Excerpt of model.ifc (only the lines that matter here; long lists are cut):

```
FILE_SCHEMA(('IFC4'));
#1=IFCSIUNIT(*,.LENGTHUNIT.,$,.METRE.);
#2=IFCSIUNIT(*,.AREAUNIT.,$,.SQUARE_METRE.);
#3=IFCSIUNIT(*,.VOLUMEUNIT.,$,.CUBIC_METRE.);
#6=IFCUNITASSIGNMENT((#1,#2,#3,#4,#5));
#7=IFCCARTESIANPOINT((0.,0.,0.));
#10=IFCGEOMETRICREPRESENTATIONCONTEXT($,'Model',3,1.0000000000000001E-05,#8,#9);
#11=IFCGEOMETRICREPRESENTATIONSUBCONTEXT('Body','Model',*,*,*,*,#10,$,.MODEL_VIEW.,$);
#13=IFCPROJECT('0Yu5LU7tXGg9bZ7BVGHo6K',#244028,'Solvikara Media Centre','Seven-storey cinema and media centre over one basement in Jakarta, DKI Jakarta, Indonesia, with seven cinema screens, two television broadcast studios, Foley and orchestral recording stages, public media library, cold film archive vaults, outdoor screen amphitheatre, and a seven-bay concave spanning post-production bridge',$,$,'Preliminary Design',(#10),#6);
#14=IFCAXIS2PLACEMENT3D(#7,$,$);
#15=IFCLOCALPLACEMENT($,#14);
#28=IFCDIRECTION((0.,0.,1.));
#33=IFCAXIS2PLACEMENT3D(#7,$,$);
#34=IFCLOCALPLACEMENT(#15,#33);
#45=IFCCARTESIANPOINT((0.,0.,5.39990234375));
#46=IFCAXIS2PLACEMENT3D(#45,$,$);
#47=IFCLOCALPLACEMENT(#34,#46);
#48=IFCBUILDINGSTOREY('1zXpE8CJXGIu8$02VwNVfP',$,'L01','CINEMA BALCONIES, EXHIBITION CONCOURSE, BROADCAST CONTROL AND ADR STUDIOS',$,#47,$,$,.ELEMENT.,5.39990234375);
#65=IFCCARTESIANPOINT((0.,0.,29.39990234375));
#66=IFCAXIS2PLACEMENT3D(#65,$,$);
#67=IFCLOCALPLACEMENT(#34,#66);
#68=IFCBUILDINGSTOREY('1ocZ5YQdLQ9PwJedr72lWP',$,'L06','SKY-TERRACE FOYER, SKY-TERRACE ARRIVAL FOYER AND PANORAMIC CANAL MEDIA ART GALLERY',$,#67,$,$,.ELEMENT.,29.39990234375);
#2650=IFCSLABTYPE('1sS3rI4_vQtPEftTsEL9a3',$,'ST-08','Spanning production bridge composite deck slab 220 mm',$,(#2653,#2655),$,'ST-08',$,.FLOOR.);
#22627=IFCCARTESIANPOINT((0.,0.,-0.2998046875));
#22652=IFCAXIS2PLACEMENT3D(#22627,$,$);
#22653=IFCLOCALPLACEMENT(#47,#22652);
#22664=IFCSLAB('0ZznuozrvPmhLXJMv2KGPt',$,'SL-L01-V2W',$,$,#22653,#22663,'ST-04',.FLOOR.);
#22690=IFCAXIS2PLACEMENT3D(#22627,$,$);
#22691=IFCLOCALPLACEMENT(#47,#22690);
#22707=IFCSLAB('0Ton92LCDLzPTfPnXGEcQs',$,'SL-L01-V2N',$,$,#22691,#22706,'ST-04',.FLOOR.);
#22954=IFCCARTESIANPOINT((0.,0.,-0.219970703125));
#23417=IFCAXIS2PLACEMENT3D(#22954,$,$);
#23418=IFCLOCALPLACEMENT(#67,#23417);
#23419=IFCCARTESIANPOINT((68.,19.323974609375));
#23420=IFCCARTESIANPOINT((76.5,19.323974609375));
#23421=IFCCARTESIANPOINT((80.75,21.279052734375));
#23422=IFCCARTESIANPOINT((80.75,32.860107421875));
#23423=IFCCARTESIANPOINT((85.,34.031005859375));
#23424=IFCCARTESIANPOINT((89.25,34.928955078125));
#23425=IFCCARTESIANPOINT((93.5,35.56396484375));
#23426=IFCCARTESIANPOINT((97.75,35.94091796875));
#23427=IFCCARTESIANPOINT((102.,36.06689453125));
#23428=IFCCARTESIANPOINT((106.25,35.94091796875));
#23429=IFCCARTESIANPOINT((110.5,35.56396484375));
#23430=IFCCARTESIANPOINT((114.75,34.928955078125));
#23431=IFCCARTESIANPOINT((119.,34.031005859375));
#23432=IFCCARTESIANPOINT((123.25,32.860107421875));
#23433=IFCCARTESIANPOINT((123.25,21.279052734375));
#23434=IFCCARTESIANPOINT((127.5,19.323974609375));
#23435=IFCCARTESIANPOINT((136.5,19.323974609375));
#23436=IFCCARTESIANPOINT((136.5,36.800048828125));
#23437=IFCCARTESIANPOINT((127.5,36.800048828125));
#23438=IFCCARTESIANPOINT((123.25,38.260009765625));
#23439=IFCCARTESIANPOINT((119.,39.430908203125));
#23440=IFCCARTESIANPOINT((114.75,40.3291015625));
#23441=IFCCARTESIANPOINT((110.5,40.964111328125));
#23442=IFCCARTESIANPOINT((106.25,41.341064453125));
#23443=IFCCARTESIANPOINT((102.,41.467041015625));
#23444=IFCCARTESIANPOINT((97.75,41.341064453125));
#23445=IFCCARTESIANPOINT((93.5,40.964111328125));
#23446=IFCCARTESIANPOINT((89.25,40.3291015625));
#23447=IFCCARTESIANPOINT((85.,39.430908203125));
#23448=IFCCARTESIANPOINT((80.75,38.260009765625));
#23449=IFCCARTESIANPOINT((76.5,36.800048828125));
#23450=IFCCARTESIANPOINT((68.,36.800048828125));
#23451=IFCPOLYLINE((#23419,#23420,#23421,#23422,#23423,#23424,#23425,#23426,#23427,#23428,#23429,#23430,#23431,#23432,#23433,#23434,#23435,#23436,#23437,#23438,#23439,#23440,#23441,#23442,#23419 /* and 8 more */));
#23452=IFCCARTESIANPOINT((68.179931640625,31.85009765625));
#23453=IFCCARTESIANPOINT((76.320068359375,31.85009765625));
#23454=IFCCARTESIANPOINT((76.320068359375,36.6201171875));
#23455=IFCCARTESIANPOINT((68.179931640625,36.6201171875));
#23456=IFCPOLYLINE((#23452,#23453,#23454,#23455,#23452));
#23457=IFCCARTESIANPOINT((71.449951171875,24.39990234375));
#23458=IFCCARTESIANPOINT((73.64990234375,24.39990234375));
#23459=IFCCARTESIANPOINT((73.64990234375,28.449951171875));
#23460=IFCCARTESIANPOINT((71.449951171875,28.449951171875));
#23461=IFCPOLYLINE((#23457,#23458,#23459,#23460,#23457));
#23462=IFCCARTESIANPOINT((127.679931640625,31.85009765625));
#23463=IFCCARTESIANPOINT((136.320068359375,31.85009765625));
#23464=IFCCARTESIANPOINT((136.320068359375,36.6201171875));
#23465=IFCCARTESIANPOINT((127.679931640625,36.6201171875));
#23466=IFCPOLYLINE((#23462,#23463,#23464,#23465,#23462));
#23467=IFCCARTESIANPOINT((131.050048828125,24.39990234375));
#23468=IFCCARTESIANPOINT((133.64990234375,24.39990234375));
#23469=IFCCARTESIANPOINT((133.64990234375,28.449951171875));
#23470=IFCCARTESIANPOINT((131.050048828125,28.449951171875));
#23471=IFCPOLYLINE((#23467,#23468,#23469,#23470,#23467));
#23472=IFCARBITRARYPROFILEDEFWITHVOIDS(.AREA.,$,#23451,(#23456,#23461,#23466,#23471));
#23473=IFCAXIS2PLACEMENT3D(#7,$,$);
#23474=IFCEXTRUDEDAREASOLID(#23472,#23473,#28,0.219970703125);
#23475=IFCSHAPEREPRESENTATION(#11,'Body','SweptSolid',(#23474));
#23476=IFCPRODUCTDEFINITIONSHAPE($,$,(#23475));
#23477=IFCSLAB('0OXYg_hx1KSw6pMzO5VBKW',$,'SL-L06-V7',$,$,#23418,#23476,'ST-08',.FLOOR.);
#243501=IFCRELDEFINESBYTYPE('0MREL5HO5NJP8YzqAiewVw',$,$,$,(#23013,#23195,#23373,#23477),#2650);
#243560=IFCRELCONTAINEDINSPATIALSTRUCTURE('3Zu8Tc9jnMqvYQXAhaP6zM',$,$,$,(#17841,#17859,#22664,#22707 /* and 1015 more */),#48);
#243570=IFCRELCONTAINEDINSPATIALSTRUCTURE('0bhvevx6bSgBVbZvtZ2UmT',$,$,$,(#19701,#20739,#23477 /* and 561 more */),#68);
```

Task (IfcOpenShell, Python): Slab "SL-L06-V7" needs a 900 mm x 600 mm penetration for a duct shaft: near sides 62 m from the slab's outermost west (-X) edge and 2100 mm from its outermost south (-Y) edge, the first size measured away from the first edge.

```python
import numpy as np
import ifcopenshell
import ifcopenshell.api.feature
import ifcopenshell.api.geometry
import ifcopenshell.api.root
import ifcopenshell.geom
import ifcopenshell.util.placement
import ifcopenshell.util.representation
import ifcopenshell.util.shape
import ifcopenshell.util.unit

model = ifcopenshell.open("model.ifc")
unit_scale = ifcopenshell.util.unit.calculate_unit_scale(model)
settings = ifcopenshell.geom.settings()


def volume(element):
    """Net volume in cubic metres, openings subtracted."""
    shape = ifcopenshell.geom.create_shape(settings, element)
    return ifcopenshell.util.shape.get_volume(shape.geometry)


slab = model.by_guid("0OXYg_hx1KSw6pMzO5VBKW")
before = volume(slab)

# Extent in the slab's own axes, in metres. The edges named are its -X and -Y sides.
slab_shape = ifcopenshell.geom.create_shape(settings, slab)
vertices = ifcopenshell.util.shape.get_vertices(slab_shape.geometry)
x_min, y_min, bottom = vertices.min(axis=0)
top = vertices[:, 2].max()

opening = ifcopenshell.api.root.create_entity(model, ifc_class="IfcOpeningElement", name="Duct shaft opening", predefined_type="OPENING")
context = ifcopenshell.util.representation.get_context(model, "Model", "Body", "MODEL_VIEW")
width, depth = 0.9, 0.6
outline = [(0.0, 0.0), (width, 0.0), (width, depth), (0.0, depth), (0.0, 0.0)]
# Overshoot both faces by 50 mm so the cut is clean.
shape = ifcopenshell.api.geometry.add_slab_representation(
    model, context=context, depth=top - bottom + 0.1, polyline=outline
)
ifcopenshell.api.geometry.assign_representation(model, product=opening, representation=shape)

matrix = ifcopenshell.util.placement.get_local_placement(slab.ObjectPlacement)
matrix[:, 3] = matrix @ np.append(np.array([x_min + 62, y_min + 2.1, bottom - 0.05]) / unit_scale, 1.0)
ifcopenshell.api.geometry.edit_object_placement(model, product=opening, matrix=matrix, is_si=False)
ifcopenshell.api.feature.add_feature(model, feature=opening, element=slab)

after = volume(slab)

print(f"slab volume {before:.3f} -> {after:.3f} m3")

model.write("model_edited.ifc")
```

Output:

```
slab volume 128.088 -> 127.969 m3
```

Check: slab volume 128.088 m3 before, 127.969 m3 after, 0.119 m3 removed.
